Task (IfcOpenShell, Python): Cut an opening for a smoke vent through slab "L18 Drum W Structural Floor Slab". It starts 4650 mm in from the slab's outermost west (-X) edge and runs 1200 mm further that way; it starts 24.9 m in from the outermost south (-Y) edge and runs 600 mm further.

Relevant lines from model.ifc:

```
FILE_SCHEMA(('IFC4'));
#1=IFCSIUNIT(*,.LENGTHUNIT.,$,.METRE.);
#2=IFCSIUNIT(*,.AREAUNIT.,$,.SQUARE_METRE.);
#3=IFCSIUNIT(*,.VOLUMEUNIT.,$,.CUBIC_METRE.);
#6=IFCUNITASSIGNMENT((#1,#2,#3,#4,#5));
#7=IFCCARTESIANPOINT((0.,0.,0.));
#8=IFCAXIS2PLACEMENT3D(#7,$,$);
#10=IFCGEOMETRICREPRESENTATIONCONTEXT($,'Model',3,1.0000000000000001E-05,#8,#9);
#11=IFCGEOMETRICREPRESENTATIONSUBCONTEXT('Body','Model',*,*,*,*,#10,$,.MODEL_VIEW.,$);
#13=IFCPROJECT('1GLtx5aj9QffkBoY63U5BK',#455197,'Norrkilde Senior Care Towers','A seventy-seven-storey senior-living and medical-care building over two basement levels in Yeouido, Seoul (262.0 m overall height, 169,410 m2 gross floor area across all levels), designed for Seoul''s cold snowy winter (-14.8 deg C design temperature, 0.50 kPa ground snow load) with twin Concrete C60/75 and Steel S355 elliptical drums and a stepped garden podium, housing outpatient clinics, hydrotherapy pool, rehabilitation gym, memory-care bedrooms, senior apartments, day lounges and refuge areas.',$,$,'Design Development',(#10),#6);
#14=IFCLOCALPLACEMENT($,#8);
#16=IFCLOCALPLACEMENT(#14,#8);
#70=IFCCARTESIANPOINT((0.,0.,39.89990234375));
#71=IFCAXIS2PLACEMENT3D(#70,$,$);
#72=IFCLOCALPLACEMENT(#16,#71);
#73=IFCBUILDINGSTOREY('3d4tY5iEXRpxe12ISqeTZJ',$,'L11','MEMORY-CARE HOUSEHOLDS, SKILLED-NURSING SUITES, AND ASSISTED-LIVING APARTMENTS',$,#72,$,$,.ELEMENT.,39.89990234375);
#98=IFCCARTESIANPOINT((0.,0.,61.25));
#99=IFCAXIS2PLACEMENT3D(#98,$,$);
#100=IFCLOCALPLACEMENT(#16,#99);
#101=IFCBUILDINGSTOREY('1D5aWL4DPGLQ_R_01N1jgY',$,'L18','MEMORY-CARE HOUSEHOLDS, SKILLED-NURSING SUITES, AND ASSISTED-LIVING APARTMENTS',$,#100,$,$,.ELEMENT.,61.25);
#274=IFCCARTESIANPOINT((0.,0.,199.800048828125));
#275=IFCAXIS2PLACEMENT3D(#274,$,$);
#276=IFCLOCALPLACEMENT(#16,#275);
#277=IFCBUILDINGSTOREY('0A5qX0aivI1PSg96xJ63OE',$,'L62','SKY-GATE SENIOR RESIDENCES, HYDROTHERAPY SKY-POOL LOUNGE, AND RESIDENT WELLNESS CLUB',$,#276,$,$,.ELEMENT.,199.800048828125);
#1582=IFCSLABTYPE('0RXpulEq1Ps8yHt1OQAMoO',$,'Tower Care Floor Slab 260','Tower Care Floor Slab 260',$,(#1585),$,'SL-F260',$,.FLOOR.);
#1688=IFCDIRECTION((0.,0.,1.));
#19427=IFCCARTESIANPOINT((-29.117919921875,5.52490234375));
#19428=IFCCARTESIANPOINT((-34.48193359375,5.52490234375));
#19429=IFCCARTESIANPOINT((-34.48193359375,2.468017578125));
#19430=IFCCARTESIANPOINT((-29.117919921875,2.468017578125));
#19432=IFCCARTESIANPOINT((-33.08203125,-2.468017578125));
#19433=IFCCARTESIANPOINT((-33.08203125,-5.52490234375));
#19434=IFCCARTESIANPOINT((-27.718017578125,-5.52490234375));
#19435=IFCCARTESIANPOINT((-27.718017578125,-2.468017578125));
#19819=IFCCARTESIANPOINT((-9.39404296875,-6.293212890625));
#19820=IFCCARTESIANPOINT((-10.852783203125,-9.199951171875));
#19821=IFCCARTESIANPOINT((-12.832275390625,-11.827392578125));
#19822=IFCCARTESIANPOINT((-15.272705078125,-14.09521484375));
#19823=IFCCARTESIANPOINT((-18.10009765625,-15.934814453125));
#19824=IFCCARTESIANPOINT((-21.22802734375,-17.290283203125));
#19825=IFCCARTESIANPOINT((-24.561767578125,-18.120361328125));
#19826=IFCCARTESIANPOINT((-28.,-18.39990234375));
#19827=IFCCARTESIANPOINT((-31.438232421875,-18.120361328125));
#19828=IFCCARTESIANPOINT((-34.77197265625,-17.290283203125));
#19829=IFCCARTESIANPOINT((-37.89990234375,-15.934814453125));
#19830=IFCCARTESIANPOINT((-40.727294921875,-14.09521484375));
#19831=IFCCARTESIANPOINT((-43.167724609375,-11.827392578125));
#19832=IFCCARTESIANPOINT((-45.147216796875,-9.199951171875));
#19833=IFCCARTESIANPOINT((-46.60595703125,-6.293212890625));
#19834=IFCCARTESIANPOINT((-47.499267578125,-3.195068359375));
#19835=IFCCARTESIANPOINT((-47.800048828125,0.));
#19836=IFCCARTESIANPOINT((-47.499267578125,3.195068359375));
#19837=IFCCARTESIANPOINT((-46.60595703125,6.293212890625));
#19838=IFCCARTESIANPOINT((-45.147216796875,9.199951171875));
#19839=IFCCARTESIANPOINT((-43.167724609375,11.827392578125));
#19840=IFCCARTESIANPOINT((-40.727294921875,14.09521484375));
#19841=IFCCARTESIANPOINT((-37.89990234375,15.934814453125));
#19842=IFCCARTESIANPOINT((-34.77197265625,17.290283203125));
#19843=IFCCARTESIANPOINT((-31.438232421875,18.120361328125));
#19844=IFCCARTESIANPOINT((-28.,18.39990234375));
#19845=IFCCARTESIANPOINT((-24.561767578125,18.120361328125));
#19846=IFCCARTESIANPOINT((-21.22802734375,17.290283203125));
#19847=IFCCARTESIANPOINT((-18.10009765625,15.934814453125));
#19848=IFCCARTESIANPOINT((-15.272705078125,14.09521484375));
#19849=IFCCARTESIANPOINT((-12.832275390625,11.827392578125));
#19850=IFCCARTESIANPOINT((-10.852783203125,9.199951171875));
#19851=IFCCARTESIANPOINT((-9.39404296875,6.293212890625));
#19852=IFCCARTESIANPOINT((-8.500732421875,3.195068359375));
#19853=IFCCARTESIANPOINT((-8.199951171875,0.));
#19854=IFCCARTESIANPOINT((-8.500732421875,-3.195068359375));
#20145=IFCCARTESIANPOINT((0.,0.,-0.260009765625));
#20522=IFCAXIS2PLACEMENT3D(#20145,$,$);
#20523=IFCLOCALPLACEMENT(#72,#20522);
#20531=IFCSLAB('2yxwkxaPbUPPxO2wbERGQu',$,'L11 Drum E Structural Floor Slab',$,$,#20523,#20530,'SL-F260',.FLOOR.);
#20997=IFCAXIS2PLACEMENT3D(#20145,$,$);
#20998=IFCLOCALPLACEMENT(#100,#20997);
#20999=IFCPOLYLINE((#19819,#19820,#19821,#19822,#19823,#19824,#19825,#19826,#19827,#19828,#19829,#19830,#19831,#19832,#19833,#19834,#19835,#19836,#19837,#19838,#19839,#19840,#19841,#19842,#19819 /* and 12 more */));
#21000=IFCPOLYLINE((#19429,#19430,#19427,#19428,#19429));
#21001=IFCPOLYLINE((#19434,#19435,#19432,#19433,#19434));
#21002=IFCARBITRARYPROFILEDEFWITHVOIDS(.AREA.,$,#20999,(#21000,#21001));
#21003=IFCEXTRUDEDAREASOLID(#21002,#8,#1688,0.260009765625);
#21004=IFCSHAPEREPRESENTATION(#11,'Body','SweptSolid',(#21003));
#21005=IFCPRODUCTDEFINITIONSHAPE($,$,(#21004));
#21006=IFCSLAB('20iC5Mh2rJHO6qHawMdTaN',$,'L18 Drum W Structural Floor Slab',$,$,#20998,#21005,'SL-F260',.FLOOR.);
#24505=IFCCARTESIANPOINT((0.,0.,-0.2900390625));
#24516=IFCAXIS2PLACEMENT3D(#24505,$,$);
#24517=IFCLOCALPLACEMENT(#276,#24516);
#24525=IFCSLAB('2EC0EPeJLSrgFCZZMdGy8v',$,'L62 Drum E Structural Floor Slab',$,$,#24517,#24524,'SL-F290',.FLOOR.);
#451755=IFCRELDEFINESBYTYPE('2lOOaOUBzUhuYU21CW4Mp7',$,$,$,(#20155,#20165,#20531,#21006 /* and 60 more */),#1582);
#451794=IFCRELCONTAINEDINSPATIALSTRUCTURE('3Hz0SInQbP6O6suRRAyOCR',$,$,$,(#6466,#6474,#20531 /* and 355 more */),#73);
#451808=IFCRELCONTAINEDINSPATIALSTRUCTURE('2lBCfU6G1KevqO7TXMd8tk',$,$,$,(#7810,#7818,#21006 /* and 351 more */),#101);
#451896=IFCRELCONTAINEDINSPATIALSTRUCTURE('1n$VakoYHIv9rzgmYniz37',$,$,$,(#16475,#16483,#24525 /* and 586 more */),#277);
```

```python
import numpy as np
import ifcopenshell
import ifcopenshell.api.feature
import ifcopenshell.api.geometry
import ifcopenshell.api.root
import ifcopenshell.geom
import ifcopenshell.util.placement
import ifcopenshell.util.representation
import ifcopenshell.util.shape
import ifcopenshell.util.unit

model = ifcopenshell.open("model.ifc")
unit_scale = ifcopenshell.util.unit.calculate_unit_scale(model)
settings = ifcopenshell.geom.settings()


def volume(element):
    """Net volume in cubic metres, openings subtracted."""
    shape = ifcopenshell.geom.create_shape(settings, element)
    return ifcopenshell.util.shape.get_volume(shape.geometry)


slab = model.by_guid("20iC5Mh2rJHO6qHawMdTaN")
before = volume(slab)

# Extent in the slab's own axes, in metres. The edges named are its -X and -Y sides.
slab_shape = ifcopenshell.geom.create_shape(settings, slab)
vertices = ifcopenshell.util.shape.get_vertices(slab_shape.geometry)
x_min, y_min, bottom = vertices.min(axis=0)
top = vertices[:, 2].max()

opening = ifcopenshell.api.root.create_entity(model, ifc_class="IfcOpeningElement", name="Smoke vent opening", predefined_type="OPENING")
context = ifcopenshell.util.representation.get_context(model, "Model", "Body", "MODEL_VIEW")
width, depth = 1.2, 0.6
outline = [(0.0, 0.0), (width, 0.0), (width, depth), (0.0, depth), (0.0, 0.0)]
# Overshoot both faces by 50 mm so the cut is clean.
shape = ifcopenshell.api.geometry.add_slab_representation(
    model, context=context, depth=top - bottom + 0.1, polyline=outline
)
ifcopenshell.api.geometry.assign_representation(model, product=opening, representation=shape)

matrix = ifcopenshell.util.placement.get_local_placement(slab.ObjectPlacement)
matrix[:, 3] = matrix @ np.append(np.array([x_min + 4.65, y_min + 24.9, bottom - 0.05]) / unit_scale, 1.0)
ifcopenshell.api.geometry.edit_object_placement(model, product=opening, matrix=matrix, is_si=False)
ifcopenshell.api.feature.add_feature(model, feature=opening, element=slab)

after = volume(slab)

print(f"slab volume {before:.3f} -> {after:.3f} m3")

model.write("model_rev.ifc")
```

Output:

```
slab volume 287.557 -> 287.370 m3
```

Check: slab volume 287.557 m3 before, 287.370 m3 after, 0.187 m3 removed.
